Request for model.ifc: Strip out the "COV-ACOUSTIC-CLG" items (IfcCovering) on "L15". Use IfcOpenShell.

First a look at what the model holds.

```python
import ifcopenshell
import ifcopenshell.util.element

model = ifcopenshell.open("model.ifc")
print(model.schema)
storey = next(s for s in model.by_type("IfcBuildingStorey") if s.Name == "L15")
coverings = [e for e in ifcopenshell.util.element.get_decomposition(storey) if e.is_a("IfcCovering")]
seen = {}
for e in coverings:
    element_type = ifcopenshell.util.element.get_type(e)
    name = element_type.Name if element_type not in (None, e) else None
    seen[name] = seen.get(name, 0) + 1
for name, count in sorted(seen.items(), key=str):
    print(count, "x", name)
```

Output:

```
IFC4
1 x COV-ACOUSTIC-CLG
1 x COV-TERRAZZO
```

```python
import ifcopenshell
import ifcopenshell.api.root
import ifcopenshell.util.element

model = ifcopenshell.open("model.ifc")

storey = next(s for s in model.by_type("IfcBuildingStorey") if s.Name == "L15")
coverings = [e for e in ifcopenshell.util.element.get_decomposition(storey) if e.is_a("IfcCovering")]
targets = [e for e in coverings if (t := ifcopenshell.util.element.get_type(e)) not in (None, e) and t.Name == "COV-ACOUSTIC-CLG"]

for e in targets:
    ifcopenshell.api.root.remove_product(model, product=e)
print(len(targets), "removed")

model.write("model_v2.ifc")
```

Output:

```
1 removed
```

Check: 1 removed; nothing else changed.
